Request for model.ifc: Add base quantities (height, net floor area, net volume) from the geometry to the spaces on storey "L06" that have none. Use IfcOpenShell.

First a look at what the model holds.

```python
import ifcopenshell
import ifcopenshell.util.element
import ifcopenshell.util.unit

model = ifcopenshell.open("model.ifc")
print(model.schema)
for unit_type in ("LENGTHUNIT", "AREAUNIT", "VOLUMEUNIT"):
    print(unit_type, ifcopenshell.util.unit.calculate_unit_scale(model, unit_type))
storey = next(s for s in model.by_type("IfcBuildingStorey") if s.Name == "L06")
spaces = [e for e in ifcopenshell.util.element.get_decomposition(storey) if e.is_a("IfcSpace")]
for e in sorted(spaces, key=lambda e: e.id()):
    print(e.id(), e.is_a(), e.Name, list(ifcopenshell.util.element.get_psets(e, qtos_only=True)), sep=" | ")
```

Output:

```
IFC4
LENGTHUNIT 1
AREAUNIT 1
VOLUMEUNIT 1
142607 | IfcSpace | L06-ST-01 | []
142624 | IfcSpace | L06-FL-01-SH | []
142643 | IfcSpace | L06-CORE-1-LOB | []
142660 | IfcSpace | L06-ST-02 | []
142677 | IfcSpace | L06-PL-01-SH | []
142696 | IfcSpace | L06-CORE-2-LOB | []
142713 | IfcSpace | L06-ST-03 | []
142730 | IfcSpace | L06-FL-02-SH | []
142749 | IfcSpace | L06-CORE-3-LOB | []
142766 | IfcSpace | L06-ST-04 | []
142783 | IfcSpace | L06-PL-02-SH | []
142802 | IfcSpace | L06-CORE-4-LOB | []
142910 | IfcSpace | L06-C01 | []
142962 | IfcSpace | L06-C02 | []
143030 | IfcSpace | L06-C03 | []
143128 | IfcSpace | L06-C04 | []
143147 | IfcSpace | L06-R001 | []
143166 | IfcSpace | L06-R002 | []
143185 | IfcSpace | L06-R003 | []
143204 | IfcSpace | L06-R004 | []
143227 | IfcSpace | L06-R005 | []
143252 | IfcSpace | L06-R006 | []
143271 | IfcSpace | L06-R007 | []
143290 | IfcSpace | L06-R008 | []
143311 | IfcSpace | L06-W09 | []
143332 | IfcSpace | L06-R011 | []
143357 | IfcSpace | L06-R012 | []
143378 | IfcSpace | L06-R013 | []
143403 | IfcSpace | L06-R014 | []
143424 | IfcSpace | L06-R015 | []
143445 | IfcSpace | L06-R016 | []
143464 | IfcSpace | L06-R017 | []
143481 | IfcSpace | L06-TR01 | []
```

```python
import ifcopenshell
import ifcopenshell.api.pset
import ifcopenshell.geom
import ifcopenshell.util.element
import ifcopenshell.util.shape
import ifcopenshell.util.unit

model = ifcopenshell.open("model.ifc")
unit_scale = ifcopenshell.util.unit.calculate_unit_scale(model)
area_scale = ifcopenshell.util.unit.calculate_unit_scale(model, "AREAUNIT")
volume_scale = ifcopenshell.util.unit.calculate_unit_scale(model, "VOLUMEUNIT")
settings = ifcopenshell.geom.settings()

storey = next(s for s in model.by_type("IfcBuildingStorey") if s.Name == "L06")
spaces = [e for e in ifcopenshell.util.element.get_decomposition(storey) if e.is_a("IfcSpace")]

for e in sorted(spaces, key=lambda e: e.id()):
    if ifcopenshell.util.element.get_psets(e, qtos_only=True, should_inherit=False):
        continue
    # Geometry comes back in metres, in the element's own axes.
    shape = ifcopenshell.geom.create_shape(settings, e)
    values = {
        "Height": ifcopenshell.util.shape.get_z(shape.geometry) / unit_scale,
        "NetFloorArea": ifcopenshell.util.shape.get_footprint_area(shape.geometry) / area_scale,
        "NetVolume": ifcopenshell.util.shape.get_volume(shape.geometry) / volume_scale,
    }
    qto = ifcopenshell.api.pset.add_qto(model, product=e, name="Qto_SpaceBaseQuantities")
    ifcopenshell.api.pset.edit_qto(model, qto=qto, properties=values)
    print(e.id(), {k: round(v, 3) for k, v in values.items()})

model.write("model-out.ifc")
```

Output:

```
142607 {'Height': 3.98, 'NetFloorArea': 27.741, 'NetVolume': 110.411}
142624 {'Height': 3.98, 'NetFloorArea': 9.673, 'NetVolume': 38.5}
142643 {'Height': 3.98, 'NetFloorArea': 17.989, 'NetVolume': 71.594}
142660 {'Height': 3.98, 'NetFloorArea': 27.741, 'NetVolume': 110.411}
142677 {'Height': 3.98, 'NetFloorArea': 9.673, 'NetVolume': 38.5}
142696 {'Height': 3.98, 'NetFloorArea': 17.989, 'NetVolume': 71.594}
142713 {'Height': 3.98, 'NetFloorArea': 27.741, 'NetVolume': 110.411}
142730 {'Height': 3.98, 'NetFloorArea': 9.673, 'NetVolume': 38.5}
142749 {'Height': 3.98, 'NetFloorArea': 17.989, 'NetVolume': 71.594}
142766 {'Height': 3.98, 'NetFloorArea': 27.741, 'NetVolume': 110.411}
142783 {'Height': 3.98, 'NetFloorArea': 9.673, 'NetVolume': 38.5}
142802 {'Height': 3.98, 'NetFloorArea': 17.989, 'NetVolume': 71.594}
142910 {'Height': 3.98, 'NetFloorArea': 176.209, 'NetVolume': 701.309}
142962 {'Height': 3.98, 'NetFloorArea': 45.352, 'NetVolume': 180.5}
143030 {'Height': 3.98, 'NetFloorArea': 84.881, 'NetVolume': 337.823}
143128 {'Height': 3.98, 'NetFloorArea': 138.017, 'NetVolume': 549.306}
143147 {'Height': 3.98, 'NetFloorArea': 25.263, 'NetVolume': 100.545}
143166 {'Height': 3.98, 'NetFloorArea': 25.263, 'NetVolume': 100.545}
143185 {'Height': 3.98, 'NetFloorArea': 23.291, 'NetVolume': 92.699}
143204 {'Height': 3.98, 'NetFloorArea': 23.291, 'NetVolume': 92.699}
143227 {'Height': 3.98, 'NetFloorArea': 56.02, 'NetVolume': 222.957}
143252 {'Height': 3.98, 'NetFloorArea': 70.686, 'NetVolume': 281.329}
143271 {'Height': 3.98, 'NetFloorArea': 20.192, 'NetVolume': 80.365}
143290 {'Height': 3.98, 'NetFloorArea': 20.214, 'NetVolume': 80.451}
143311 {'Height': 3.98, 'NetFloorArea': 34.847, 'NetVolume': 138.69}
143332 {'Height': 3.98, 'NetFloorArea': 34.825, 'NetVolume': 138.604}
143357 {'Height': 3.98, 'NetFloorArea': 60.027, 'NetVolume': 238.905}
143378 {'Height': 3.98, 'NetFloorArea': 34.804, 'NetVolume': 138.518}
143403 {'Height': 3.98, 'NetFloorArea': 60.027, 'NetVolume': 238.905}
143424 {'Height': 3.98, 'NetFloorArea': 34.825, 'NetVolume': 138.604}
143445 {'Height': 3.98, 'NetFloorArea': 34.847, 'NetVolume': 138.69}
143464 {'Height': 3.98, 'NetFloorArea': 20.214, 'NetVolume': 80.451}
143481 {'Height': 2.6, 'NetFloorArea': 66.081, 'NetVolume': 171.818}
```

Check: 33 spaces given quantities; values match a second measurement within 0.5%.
